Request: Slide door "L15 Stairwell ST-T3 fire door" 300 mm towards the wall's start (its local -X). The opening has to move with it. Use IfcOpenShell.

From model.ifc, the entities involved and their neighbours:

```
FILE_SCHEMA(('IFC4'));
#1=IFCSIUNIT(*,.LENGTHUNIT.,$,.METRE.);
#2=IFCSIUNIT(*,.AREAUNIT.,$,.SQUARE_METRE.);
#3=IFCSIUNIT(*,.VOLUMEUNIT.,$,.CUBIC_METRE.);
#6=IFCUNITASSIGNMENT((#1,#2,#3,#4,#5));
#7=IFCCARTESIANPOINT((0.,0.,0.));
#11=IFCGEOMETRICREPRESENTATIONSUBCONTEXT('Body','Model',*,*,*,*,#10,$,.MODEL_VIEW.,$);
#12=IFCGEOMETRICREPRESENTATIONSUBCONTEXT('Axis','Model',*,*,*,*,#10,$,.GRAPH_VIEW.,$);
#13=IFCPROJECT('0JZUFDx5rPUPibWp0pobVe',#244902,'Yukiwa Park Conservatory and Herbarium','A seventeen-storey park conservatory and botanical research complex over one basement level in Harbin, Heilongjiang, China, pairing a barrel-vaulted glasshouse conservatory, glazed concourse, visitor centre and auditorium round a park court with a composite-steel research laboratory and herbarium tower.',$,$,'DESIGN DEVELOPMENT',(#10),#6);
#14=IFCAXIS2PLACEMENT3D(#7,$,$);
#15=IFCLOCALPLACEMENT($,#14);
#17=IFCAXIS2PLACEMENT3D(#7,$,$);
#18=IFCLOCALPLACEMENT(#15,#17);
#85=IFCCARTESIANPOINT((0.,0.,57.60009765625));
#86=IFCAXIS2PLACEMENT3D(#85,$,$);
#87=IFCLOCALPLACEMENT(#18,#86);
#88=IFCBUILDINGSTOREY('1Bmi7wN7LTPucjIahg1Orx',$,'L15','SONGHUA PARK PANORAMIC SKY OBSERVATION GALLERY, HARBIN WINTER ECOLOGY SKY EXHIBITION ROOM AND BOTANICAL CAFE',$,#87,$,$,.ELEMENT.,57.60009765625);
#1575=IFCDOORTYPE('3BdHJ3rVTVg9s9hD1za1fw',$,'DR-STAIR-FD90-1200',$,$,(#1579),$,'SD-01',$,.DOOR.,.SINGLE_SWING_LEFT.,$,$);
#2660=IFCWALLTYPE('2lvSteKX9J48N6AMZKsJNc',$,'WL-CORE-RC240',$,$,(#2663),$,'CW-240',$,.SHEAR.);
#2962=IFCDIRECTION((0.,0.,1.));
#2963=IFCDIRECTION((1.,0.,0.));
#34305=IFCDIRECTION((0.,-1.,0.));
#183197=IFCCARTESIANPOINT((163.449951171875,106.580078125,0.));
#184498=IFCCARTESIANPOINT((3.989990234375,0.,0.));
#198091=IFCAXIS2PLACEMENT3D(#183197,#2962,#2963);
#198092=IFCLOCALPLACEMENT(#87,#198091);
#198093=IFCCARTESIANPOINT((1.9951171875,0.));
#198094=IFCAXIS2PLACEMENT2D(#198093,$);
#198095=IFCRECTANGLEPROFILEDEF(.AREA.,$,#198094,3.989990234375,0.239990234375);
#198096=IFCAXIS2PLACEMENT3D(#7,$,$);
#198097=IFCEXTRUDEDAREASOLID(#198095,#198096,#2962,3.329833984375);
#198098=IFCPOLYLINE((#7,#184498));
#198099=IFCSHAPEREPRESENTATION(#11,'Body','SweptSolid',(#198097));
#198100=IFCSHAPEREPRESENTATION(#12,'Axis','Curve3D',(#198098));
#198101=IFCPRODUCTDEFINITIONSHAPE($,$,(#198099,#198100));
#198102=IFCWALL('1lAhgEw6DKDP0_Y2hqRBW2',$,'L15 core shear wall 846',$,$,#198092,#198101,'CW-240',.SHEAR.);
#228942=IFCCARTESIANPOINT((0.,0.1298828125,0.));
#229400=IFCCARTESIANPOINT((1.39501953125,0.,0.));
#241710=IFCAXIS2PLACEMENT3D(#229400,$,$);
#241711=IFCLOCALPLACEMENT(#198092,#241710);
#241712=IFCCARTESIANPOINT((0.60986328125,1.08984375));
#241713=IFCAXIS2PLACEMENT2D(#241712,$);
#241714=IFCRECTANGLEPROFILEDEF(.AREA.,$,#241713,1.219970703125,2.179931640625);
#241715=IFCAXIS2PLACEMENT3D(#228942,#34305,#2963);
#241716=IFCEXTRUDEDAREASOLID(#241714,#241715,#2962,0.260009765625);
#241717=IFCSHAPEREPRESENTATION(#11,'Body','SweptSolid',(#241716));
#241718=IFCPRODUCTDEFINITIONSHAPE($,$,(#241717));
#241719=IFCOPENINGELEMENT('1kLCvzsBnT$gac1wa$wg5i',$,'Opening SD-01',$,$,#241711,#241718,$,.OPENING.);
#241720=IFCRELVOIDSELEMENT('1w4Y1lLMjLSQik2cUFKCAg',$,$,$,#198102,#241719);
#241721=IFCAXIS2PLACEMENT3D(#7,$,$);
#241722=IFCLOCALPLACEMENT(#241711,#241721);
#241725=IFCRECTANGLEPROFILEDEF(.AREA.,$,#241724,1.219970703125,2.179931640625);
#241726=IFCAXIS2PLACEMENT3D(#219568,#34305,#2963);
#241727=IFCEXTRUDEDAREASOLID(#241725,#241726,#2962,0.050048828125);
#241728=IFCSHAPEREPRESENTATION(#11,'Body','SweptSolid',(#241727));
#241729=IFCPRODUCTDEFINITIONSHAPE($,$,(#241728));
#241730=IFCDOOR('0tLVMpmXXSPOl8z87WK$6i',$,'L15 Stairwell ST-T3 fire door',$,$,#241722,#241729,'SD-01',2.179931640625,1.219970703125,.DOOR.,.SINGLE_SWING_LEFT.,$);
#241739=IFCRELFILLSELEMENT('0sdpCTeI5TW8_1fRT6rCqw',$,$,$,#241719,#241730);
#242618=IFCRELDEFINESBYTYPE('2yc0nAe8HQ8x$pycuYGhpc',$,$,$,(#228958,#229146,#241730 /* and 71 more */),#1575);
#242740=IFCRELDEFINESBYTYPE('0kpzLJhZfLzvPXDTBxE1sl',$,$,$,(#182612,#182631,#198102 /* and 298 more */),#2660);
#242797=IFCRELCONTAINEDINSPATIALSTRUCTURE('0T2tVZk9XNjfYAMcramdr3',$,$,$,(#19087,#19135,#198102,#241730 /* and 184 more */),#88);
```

```python
import ifcopenshell
import ifcopenshell.api.geometry
import ifcopenshell.util.placement
import ifcopenshell.util.unit

model = ifcopenshell.open("model.ifc")
unit_scale = ifcopenshell.util.unit.calculate_unit_scale(model)

door = model.by_guid("0tLVMpmXXSPOl8z87WK$6i")
opening = door.FillsVoids[0].RelatingOpeningElement
wall = opening.VoidsElements[0].RelatingBuildingElement

wall_matrix = ifcopenshell.util.placement.get_local_placement(wall.ObjectPlacement)
shift = wall_matrix[:3, 0] * -0.3 / unit_scale
before = ifcopenshell.util.placement.get_local_placement(door.ObjectPlacement)[:3, 3].copy()

# The door is placed relative to its opening, so it follows when the opening moves.
matrix = ifcopenshell.util.placement.get_local_placement(opening.ObjectPlacement)
matrix[:3, 3] += shift
ifcopenshell.api.geometry.edit_object_placement(
    model, product=opening, matrix=matrix, is_si=False, should_transform_children=True
)

after = ifcopenshell.util.placement.get_local_placement(door.ObjectPlacement)[:3, 3]
print("door moved by", (after - before).round(3) + 0.0)

model.write("model_v2.ifc")
```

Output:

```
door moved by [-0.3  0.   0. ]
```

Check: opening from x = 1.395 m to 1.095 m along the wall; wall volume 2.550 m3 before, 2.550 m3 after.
